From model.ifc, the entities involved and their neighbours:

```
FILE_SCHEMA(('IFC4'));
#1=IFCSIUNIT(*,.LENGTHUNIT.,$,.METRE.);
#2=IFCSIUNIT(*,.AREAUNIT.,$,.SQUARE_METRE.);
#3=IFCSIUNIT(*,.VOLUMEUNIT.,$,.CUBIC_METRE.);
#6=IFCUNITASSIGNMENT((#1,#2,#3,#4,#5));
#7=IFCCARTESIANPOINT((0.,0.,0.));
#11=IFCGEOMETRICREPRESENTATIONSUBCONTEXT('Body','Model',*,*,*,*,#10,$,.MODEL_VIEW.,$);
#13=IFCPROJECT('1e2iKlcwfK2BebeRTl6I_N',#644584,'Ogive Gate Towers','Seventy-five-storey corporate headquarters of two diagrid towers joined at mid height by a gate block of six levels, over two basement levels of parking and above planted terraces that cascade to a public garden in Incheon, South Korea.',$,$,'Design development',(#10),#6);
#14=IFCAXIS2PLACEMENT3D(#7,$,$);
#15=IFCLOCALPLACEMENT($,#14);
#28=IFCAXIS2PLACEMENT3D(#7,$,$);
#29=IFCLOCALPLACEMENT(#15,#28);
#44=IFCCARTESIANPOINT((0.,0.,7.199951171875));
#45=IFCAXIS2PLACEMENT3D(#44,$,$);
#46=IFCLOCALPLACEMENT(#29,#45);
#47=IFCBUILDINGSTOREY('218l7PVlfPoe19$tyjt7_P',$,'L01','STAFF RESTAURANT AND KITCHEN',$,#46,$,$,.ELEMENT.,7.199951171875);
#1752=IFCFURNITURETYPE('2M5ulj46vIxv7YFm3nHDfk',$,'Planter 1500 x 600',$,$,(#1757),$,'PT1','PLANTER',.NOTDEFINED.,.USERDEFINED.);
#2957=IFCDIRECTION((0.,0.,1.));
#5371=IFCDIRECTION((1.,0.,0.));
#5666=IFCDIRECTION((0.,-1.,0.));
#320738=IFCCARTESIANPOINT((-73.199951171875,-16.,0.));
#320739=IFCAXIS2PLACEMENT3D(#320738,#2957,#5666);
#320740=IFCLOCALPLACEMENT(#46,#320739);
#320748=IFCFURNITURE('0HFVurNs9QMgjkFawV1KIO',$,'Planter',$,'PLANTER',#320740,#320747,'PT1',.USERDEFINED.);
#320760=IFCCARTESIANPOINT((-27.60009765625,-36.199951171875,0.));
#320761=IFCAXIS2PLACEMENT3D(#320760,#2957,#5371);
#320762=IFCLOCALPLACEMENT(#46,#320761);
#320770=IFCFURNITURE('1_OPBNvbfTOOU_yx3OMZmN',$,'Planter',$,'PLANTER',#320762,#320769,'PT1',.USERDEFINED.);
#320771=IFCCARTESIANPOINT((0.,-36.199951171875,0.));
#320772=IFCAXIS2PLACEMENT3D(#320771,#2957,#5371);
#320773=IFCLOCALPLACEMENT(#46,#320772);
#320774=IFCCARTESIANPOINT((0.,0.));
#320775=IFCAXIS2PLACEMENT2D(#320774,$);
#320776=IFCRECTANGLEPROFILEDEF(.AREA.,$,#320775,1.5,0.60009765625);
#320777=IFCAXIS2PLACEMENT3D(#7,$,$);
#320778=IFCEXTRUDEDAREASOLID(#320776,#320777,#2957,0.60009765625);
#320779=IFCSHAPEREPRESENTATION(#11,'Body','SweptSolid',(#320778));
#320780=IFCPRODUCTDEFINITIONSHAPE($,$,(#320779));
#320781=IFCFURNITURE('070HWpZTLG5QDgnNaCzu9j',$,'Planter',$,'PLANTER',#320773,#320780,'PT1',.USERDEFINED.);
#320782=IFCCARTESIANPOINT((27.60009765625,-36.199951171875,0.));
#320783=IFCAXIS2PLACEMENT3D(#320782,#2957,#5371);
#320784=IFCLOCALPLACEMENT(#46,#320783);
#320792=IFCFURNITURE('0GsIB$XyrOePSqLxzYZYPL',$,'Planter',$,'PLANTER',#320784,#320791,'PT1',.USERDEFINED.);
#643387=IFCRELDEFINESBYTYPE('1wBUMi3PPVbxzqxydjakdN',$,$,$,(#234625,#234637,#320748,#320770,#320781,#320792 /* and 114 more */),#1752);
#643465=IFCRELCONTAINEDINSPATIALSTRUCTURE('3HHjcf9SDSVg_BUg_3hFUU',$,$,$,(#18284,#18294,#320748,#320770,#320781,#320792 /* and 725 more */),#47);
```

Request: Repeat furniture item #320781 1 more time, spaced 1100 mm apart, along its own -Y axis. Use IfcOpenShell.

```python
import ifcopenshell
import ifcopenshell.api.geometry
import ifcopenshell.api.root
import ifcopenshell.util.element
import ifcopenshell.util.placement

model = ifcopenshell.open("model.ifc")

source = model.by_id(320781)
base = ifcopenshell.util.placement.get_local_placement(source.ObjectPlacement)
step = -base[:3, 1] * 1.1

for i in range(1, 2):
    copy = ifcopenshell.api.root.copy_class(model, product=source)
    copy.Representation = ifcopenshell.util.element.copy_deep(
        model, source.Representation, exclude=["IfcGeometricRepresentationContext", "IfcRepresentationMap"]
    )
    copy.Tag = None
    matrix = base.copy()
    matrix[:3, 3] += i * step
    print("added at", matrix[:3, 3].round(3) + 0.0)
    ifcopenshell.api.geometry.edit_object_placement(model, product=copy, matrix=matrix, is_si=False)

model.write("model_v2.ifc")
```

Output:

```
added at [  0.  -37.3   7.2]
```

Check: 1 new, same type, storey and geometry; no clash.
